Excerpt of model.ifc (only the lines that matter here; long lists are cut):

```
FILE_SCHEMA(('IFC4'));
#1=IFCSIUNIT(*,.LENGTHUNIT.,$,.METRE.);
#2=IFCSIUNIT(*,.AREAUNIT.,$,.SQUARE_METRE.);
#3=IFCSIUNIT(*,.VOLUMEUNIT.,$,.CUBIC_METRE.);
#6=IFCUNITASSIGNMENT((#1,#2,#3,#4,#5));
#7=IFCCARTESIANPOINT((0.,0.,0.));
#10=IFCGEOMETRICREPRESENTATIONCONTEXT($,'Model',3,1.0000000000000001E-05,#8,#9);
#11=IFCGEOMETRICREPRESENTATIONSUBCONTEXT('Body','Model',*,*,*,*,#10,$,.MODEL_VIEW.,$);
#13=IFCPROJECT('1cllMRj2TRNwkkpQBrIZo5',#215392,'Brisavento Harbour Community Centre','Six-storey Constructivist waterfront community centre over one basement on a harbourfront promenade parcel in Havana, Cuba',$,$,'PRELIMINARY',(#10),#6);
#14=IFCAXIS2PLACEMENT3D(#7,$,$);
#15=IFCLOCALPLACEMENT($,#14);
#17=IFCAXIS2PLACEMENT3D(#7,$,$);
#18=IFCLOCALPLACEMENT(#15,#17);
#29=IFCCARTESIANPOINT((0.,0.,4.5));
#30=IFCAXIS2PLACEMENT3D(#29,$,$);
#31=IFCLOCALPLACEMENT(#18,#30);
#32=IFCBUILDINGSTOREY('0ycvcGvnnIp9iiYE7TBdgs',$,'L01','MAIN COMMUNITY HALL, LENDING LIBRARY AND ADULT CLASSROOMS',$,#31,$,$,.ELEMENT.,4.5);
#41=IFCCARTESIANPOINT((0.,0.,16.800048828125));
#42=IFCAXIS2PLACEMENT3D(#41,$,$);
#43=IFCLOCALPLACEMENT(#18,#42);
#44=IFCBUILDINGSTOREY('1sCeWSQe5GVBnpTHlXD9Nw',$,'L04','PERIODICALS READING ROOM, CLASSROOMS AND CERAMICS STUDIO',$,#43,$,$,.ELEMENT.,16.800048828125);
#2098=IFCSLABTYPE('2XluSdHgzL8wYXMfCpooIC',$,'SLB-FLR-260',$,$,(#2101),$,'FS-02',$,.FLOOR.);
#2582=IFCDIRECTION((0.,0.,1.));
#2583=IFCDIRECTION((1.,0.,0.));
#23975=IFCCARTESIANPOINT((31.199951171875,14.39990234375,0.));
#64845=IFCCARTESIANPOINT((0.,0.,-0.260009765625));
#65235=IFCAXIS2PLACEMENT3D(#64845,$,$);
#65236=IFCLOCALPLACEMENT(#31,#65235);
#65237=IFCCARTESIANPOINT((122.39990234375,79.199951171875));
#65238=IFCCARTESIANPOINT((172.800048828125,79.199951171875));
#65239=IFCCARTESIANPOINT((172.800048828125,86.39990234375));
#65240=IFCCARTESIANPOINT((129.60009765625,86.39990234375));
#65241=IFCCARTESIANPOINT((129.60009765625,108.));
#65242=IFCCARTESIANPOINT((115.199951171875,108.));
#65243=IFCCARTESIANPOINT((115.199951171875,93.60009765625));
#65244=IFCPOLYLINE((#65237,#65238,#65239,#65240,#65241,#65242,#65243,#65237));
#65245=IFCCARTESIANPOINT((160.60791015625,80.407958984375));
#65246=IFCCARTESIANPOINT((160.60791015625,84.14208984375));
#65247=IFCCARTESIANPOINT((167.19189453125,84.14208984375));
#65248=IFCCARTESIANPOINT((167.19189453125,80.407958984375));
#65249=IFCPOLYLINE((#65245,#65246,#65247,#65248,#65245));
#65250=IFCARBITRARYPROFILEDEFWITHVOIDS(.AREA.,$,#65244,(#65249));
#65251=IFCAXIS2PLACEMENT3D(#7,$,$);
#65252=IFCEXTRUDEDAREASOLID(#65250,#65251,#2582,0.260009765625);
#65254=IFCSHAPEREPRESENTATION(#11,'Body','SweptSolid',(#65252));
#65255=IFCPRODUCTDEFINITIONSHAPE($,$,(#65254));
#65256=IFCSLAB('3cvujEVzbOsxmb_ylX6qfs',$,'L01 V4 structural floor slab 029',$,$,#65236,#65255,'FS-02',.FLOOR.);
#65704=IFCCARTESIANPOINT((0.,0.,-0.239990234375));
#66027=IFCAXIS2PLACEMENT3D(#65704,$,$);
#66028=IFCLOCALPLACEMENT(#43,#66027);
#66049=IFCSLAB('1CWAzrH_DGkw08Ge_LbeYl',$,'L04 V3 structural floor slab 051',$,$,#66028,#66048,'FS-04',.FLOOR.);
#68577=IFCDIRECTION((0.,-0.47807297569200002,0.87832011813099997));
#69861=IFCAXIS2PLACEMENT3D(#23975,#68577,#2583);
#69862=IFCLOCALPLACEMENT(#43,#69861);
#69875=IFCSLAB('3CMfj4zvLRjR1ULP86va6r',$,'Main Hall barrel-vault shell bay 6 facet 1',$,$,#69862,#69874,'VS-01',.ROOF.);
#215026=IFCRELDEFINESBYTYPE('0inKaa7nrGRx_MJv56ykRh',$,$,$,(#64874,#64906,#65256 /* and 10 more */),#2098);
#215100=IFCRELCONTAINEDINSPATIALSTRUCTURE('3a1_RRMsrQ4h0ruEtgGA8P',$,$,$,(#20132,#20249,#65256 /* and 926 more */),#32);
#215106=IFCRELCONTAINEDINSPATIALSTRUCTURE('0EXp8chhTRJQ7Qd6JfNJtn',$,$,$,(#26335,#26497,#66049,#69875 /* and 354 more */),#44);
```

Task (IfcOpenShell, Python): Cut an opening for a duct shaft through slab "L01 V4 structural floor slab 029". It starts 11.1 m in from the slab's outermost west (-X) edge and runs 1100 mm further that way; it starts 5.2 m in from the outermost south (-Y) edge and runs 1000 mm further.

```python
import numpy as np
import ifcopenshell
import ifcopenshell.api.feature
import ifcopenshell.api.geometry
import ifcopenshell.api.root
import ifcopenshell.geom
import ifcopenshell.util.placement
import ifcopenshell.util.representation
import ifcopenshell.util.shape
import ifcopenshell.util.unit

model = ifcopenshell.open("model.ifc")
unit_scale = ifcopenshell.util.unit.calculate_unit_scale(model)
settings = ifcopenshell.geom.settings()


def volume(element):
    """Net volume in cubic metres, openings subtracted."""
    shape = ifcopenshell.geom.create_shape(settings, element)
    return ifcopenshell.util.shape.get_volume(shape.geometry)


slab = model.by_guid("3cvujEVzbOsxmb_ylX6qfs")
before = volume(slab)

# Extent in the slab's own axes, in metres. The edges named are its -X and -Y sides.
slab_shape = ifcopenshell.geom.create_shape(settings, slab)
vertices = ifcopenshell.util.shape.get_vertices(slab_shape.geometry)
x_min, y_min, bottom = vertices.min(axis=0)
top = vertices[:, 2].max()

opening = ifcopenshell.api.root.create_entity(model, ifc_class="IfcOpeningElement", name="Duct shaft opening", predefined_type="OPENING")
context = ifcopenshell.util.representation.get_context(model, "Model", "Body", "MODEL_VIEW")
width, depth = 1.1, 1
outline = [(0.0, 0.0), (width, 0.0), (width, depth), (0.0, depth), (0.0, 0.0)]
# Overshoot both faces by 50 mm so the cut is clean.
shape = ifcopenshell.api.geometry.add_slab_representation(
    model, context=context, depth=top - bottom + 0.1, polyline=outline
)
ifcopenshell.api.geometry.assign_representation(model, product=opening, representation=shape)

matrix = ifcopenshell.util.placement.get_local_placement(slab.ObjectPlacement)
matrix[:, 3] = matrix @ np.append(np.array([x_min + 11.1, y_min + 5.2, bottom - 0.05]) / unit_scale, 1.0)
ifcopenshell.api.geometry.edit_object_placement(model, product=opening, matrix=matrix, is_si=False)
ifcopenshell.api.feature.add_feature(model, feature=opening, element=slab)

after = volume(slab)

print(f"slab volume {before:.3f} -> {after:.3f} m3")

model.write("model_edited.ifc")
```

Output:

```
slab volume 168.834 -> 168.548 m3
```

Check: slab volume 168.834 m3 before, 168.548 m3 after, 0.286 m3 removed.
